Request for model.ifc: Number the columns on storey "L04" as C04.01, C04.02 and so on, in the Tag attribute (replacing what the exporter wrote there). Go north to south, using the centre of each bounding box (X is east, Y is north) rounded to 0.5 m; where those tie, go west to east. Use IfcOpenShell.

First a look at what the model holds.

```python
import ifcopenshell
import ifcopenshell.util.element
import ifcopenshell.util.placement

model = ifcopenshell.open("model.ifc")
print(model.schema)
storey = next(s for s in model.by_type("IfcBuildingStorey") if s.Name == "L04")
columns = [e for e in ifcopenshell.util.element.get_decomposition(storey) if e.is_a("IfcColumn")]
for e in sorted(columns, key=lambda e: e.id()):
    origin = ifcopenshell.util.placement.get_local_placement(e.ObjectPlacement)[:3, 3]
    print(e.id(), e.Tag, e.Name, origin.round(2) + 0.0, sep=" | ")
```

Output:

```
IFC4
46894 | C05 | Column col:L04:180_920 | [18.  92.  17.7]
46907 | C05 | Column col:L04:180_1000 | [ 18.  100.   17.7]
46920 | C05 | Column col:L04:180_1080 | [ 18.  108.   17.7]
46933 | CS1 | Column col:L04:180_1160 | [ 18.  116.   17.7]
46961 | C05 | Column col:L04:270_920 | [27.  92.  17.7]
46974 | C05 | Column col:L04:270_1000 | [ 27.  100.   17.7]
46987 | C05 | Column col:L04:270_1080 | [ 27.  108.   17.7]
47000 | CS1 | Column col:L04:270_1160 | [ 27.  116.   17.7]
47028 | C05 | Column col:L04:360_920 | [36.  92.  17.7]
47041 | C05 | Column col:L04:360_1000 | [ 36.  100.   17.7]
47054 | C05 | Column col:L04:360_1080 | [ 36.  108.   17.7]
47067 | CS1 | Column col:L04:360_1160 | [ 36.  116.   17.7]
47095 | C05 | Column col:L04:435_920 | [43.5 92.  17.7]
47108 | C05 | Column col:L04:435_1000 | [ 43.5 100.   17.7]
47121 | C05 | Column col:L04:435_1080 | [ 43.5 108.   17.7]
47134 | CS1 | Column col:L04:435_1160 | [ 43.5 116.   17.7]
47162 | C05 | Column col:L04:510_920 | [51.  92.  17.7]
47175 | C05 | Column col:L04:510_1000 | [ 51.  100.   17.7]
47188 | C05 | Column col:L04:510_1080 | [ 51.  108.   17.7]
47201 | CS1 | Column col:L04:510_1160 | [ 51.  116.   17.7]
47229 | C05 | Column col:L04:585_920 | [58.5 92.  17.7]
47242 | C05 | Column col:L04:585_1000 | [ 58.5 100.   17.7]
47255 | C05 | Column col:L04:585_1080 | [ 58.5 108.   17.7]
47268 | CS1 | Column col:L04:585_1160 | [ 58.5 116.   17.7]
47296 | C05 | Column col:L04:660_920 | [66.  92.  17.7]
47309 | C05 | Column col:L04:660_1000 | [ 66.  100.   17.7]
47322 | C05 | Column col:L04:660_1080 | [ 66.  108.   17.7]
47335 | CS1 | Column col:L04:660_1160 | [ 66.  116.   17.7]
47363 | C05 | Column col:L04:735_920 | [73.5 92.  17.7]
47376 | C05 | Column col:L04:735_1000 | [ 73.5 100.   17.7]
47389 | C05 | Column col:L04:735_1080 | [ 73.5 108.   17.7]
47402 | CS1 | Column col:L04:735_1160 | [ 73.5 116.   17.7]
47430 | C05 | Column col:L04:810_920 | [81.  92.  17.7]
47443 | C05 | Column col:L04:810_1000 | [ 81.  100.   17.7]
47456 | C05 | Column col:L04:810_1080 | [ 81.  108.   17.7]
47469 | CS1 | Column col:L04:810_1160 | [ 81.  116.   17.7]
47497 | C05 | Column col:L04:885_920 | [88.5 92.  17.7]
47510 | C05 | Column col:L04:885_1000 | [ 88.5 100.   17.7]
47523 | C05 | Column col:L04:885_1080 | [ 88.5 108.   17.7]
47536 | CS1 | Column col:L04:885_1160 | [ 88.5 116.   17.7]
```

```python
import ifcopenshell
import ifcopenshell.geom
import ifcopenshell.util.element
import ifcopenshell.util.shape

model = ifcopenshell.open("model.ifc")
settings = ifcopenshell.geom.settings()
settings.set("use-world-coords", True)


def centre(element):
    shape = ifcopenshell.geom.create_shape(settings, element)
    return ifcopenshell.util.shape.get_bbox_centroid(shape.geometry)


storey = next(s for s in model.by_type("IfcBuildingStorey") if s.Name == "L04")
columns = [e for e in ifcopenshell.util.element.get_decomposition(storey) if e.is_a("IfcColumn")]

# Insertion points can sit at a corner or the storey origin, so sort by the geometry (in metres).
centres = {e: centre(e) for e in columns}
columns.sort(key=lambda e: (-round(centres[e][1] / 0.5), centres[e][0]))

for i, e in enumerate(columns, start=1):
    number = f"C04.{i:02d}"
    e.Tag = number
    print(e.id(), number)

model.write("model_updated.ifc")
```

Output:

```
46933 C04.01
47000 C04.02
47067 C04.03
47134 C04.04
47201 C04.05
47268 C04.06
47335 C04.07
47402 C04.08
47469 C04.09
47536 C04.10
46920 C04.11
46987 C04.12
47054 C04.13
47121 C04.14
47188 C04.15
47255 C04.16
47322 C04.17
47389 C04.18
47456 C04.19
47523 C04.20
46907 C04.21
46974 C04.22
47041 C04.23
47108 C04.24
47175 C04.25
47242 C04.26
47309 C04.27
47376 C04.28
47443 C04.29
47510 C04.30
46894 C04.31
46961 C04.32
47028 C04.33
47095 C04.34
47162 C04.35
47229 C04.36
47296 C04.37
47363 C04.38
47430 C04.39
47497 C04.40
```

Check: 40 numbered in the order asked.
